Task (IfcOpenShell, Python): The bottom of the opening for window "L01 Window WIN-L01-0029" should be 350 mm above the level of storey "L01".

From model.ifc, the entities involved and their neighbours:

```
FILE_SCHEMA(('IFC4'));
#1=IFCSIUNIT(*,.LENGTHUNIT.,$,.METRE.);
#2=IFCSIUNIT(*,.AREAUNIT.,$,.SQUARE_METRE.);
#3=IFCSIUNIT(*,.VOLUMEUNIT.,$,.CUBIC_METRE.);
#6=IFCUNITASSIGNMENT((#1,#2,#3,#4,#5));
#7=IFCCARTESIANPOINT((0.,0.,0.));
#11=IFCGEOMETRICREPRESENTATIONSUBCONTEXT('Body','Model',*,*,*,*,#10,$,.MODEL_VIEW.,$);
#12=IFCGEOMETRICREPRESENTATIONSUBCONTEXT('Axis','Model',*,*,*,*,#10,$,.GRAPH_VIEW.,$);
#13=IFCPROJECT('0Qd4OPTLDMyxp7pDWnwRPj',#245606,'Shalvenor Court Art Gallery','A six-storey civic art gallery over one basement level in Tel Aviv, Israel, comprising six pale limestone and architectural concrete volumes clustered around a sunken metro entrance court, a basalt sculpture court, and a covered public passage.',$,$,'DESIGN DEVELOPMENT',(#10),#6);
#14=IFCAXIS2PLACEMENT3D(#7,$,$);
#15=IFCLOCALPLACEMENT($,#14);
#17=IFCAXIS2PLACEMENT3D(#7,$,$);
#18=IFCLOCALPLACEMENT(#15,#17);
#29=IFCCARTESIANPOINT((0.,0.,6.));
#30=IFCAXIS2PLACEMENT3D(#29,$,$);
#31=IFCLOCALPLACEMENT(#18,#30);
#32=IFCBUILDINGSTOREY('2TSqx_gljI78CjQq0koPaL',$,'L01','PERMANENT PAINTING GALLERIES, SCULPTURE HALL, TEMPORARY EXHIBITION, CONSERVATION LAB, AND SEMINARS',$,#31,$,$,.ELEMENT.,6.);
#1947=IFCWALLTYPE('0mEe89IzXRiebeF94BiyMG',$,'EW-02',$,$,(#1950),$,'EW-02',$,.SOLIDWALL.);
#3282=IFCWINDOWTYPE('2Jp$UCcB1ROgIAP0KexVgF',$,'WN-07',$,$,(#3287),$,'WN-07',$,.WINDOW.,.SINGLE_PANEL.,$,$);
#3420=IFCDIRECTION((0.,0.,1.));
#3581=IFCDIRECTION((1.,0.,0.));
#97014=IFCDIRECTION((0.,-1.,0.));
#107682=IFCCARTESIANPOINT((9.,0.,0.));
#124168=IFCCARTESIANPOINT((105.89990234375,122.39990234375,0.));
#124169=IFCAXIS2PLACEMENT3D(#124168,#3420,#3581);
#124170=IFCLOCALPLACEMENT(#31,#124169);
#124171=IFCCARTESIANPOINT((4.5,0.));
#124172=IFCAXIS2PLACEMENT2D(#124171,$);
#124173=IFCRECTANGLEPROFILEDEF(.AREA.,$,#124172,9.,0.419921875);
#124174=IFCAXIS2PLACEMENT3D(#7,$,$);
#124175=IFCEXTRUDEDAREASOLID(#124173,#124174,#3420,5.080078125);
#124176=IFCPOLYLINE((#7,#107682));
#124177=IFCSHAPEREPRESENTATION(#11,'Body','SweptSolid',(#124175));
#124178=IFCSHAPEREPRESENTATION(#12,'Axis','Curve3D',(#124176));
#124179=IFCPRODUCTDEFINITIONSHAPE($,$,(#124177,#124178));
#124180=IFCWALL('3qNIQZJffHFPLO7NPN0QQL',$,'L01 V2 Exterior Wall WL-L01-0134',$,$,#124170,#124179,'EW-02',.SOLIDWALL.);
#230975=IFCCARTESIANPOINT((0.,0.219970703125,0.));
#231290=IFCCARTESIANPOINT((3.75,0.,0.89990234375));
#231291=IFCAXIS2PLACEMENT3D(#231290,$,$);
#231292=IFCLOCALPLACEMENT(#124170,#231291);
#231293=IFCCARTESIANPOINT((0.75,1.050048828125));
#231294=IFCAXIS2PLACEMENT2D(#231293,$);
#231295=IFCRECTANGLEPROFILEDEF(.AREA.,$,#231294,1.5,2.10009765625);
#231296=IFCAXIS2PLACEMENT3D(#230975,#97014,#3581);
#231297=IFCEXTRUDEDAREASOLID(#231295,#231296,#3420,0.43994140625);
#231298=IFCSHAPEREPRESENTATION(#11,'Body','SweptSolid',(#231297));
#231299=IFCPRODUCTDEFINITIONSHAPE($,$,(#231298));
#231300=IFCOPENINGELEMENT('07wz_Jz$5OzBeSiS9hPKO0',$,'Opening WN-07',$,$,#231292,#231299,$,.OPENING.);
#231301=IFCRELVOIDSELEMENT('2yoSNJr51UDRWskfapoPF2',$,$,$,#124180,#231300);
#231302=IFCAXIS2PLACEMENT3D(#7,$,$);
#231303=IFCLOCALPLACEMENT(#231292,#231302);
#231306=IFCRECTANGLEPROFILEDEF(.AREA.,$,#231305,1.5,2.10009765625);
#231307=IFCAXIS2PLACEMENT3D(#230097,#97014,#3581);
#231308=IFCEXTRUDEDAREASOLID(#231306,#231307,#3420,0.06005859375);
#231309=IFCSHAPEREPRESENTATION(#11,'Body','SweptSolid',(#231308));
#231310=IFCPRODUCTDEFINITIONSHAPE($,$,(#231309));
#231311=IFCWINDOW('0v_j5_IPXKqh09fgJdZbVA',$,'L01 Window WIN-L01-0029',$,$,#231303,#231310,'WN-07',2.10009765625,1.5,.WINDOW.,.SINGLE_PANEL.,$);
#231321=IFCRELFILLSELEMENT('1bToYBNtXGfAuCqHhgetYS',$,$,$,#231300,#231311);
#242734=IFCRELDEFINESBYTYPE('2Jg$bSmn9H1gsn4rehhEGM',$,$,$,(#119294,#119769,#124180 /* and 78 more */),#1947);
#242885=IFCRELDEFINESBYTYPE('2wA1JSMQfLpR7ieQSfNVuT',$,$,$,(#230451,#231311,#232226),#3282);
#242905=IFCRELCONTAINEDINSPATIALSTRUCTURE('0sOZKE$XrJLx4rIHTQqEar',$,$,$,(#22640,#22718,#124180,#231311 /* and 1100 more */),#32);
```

```python
import numpy as np
import ifcopenshell
import ifcopenshell.api.geometry
import ifcopenshell.geom
import ifcopenshell.util.element
import ifcopenshell.util.placement
import ifcopenshell.util.shape
import ifcopenshell.util.unit

model = ifcopenshell.open("model.ifc")
unit_scale = ifcopenshell.util.unit.calculate_unit_scale(model)

window = model.by_guid("0v_j5_IPXKqh09fgJdZbVA")
opening = window.FillsVoids[0].RelatingOpeningElement
storey = ifcopenshell.util.element.get_container(window, ifc_class="IfcBuildingStorey")
level = ifcopenshell.util.placement.get_local_placement(storey.ObjectPlacement)[2, 3]

# The opening's origin need not be at the sill, so measure its lowest point.
shape = ifcopenshell.geom.create_shape(ifcopenshell.geom.settings(), opening)
bottom = ifcopenshell.util.shape.get_shape_bottom_elevation(shape, shape.geometry) / unit_scale
dz = level + 0.35 / unit_scale - bottom

shift = np.array([0.0, 0.0, dz])
# The window is placed relative to its opening, so it follows when the opening moves.
matrix = ifcopenshell.util.placement.get_local_placement(opening.ObjectPlacement)
matrix[:3, 3] += shift
ifcopenshell.api.geometry.edit_object_placement(
    model, product=opening, matrix=matrix, is_si=False, should_transform_children=True
)

print(f"moved by {dz * unit_scale:+.3f} m")

model.write("model_v2.ifc")
```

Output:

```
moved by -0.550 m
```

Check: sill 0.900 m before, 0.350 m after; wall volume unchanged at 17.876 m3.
